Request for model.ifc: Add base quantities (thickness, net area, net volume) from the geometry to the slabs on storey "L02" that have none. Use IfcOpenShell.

First a look at what the model holds.

```python
import ifcopenshell
import ifcopenshell.util.element
import ifcopenshell.util.unit

model = ifcopenshell.open("model.ifc")
print(model.schema)
for unit_type in ("LENGTHUNIT", "AREAUNIT", "VOLUMEUNIT"):
    print(unit_type, ifcopenshell.util.unit.calculate_unit_scale(model, unit_type))
storey = next(s for s in model.by_type("IfcBuildingStorey") if s.Name == "L02")
slabs = [e for e in ifcopenshell.util.element.get_decomposition(storey) if e.is_a("IfcSlab")]
for e in sorted(slabs, key=lambda e: e.id()):
    print(e.id(), e.is_a(), e.Name, list(ifcopenshell.util.element.get_psets(e, qtos_only=True)), sep=" | ")
```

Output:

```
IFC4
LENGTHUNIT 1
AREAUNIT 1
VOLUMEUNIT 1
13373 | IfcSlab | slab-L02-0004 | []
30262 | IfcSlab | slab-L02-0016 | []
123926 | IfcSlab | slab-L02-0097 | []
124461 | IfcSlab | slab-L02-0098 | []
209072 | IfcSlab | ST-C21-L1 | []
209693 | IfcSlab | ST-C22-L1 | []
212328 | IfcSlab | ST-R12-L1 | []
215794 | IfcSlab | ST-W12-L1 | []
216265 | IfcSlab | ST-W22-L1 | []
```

```python
import ifcopenshell
import ifcopenshell.api.pset
import ifcopenshell.geom
import ifcopenshell.util.element
import ifcopenshell.util.shape
import ifcopenshell.util.unit

model = ifcopenshell.open("model.ifc")
unit_scale = ifcopenshell.util.unit.calculate_unit_scale(model)
area_scale = ifcopenshell.util.unit.calculate_unit_scale(model, "AREAUNIT")
volume_scale = ifcopenshell.util.unit.calculate_unit_scale(model, "VOLUMEUNIT")
settings = ifcopenshell.geom.settings()

storey = next(s for s in model.by_type("IfcBuildingStorey") if s.Name == "L02")
slabs = [e for e in ifcopenshell.util.element.get_decomposition(storey) if e.is_a("IfcSlab")]

for e in sorted(slabs, key=lambda e: e.id()):
    if ifcopenshell.util.element.get_psets(e, qtos_only=True, should_inherit=False):
        continue
    # Geometry comes back in metres, in the element's own axes.
    shape = ifcopenshell.geom.create_shape(settings, e)
    values = {
        "Width": ifcopenshell.util.shape.get_z(shape.geometry) / unit_scale,
        "NetArea": ifcopenshell.util.shape.get_footprint_area(shape.geometry) / area_scale,
        "NetVolume": ifcopenshell.util.shape.get_volume(shape.geometry) / volume_scale,
    }
    qto = ifcopenshell.api.pset.add_qto(model, product=e, name="Qto_SlabBaseQuantities")
    ifcopenshell.api.pset.edit_qto(model, qto=qto, properties=values)
    print(e.id(), {k: round(v, 3) for k, v in values.items()})

model.write("model_updated.ifc")
```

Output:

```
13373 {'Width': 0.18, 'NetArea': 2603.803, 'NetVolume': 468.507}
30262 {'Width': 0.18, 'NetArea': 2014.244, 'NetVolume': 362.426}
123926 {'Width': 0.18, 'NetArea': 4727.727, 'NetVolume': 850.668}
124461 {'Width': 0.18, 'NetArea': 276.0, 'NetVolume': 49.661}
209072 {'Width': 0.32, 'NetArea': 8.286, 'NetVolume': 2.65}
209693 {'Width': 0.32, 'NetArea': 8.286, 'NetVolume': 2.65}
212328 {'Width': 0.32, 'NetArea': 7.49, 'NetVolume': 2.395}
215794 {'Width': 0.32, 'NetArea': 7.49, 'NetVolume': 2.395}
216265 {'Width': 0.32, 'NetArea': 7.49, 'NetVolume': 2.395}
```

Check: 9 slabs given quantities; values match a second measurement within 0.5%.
